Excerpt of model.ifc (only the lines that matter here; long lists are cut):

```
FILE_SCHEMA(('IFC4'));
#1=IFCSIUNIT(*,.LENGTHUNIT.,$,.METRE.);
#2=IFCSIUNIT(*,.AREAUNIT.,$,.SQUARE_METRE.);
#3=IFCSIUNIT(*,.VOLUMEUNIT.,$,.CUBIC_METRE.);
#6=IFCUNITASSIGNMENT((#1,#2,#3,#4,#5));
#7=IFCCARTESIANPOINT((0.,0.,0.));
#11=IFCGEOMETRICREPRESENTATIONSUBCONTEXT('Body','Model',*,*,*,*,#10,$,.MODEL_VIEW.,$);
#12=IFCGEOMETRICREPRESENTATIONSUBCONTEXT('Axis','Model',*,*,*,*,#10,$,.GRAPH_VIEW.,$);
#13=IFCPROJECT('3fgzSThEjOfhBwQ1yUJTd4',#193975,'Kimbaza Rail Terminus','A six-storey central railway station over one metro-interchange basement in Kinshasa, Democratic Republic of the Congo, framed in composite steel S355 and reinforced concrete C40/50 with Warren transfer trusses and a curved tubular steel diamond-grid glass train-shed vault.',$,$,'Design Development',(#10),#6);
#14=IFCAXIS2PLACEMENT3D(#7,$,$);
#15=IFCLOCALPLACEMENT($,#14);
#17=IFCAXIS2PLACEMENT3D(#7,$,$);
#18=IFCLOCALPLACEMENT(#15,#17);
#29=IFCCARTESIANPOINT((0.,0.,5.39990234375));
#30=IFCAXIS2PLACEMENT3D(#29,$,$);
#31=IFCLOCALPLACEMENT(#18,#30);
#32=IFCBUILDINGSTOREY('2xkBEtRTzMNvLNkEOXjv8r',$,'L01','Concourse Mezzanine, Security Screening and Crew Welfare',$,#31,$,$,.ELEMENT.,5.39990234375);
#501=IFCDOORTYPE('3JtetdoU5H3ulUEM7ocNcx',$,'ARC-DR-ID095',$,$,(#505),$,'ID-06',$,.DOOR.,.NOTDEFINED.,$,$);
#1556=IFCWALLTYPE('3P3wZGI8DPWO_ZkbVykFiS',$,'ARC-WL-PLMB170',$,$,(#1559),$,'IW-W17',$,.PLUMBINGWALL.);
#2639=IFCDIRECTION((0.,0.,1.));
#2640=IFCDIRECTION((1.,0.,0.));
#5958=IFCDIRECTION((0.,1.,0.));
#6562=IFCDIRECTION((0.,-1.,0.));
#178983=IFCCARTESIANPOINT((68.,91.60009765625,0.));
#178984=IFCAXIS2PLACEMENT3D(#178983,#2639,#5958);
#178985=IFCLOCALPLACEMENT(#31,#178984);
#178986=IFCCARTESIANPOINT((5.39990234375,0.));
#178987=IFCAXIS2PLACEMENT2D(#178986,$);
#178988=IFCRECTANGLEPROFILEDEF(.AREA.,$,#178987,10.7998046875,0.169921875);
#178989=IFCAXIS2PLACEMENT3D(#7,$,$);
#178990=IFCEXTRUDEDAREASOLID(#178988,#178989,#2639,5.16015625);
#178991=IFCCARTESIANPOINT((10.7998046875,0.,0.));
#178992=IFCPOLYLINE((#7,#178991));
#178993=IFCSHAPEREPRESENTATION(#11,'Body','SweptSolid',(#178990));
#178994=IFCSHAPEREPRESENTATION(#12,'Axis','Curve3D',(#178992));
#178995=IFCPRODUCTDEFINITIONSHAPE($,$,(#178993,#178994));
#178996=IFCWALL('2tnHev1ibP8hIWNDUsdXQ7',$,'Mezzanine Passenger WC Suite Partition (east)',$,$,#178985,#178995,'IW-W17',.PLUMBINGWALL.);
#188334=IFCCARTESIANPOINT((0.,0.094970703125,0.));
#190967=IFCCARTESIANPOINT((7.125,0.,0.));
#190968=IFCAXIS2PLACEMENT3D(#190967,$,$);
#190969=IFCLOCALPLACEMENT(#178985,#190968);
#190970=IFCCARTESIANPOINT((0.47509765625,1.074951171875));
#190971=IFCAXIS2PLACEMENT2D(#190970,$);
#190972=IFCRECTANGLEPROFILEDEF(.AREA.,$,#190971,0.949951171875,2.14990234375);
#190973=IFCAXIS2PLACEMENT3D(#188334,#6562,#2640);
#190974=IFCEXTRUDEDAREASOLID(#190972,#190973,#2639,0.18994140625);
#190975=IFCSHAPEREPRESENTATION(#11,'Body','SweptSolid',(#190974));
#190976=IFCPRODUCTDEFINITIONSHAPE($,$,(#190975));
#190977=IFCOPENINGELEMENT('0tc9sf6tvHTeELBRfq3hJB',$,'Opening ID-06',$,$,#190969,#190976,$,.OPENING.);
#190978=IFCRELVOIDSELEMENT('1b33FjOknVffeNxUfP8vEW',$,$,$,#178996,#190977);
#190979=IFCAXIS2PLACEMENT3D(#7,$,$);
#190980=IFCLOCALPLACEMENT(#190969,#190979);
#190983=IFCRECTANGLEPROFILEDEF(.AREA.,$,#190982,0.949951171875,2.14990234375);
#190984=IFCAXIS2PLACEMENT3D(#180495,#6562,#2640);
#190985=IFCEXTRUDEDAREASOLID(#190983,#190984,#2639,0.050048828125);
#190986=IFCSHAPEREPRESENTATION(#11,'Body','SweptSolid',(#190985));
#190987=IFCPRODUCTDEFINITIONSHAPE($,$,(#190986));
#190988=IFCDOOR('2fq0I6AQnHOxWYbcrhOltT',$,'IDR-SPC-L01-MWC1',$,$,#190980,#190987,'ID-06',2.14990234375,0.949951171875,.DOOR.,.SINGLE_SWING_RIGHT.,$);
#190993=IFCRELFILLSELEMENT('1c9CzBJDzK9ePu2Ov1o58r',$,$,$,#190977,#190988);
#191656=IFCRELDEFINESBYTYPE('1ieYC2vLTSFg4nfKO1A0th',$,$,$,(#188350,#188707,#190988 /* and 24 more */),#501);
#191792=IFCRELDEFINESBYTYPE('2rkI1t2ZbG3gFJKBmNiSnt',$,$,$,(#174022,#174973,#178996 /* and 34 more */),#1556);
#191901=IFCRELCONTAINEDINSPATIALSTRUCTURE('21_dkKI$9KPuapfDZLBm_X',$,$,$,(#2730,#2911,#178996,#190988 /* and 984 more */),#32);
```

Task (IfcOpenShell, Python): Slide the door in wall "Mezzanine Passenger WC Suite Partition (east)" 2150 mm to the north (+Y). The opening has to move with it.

```python
import ifcopenshell
import ifcopenshell.api.geometry
import ifcopenshell.util.placement

model = ifcopenshell.open("model.ifc")

door = model.by_guid("2fq0I6AQnHOxWYbcrhOltT")
opening = door.FillsVoids[0].RelatingOpeningElement
wall = opening.VoidsElements[0].RelatingBuildingElement

wall_matrix = ifcopenshell.util.placement.get_local_placement(wall.ObjectPlacement)
shift = wall_matrix[:3, 0] * 2.15
before = ifcopenshell.util.placement.get_local_placement(door.ObjectPlacement)[:3, 3].copy()

# The door is placed relative to its opening, so it follows when the opening moves.
matrix = ifcopenshell.util.placement.get_local_placement(opening.ObjectPlacement)
matrix[:3, 3] += shift
ifcopenshell.api.geometry.edit_object_placement(
    model, product=opening, matrix=matrix, is_si=False, should_transform_children=True
)

after = ifcopenshell.util.placement.get_local_placement(door.ObjectPlacement)[:3, 3]
print("door moved by", (after - before).round(3) + 0.0)

model.write("model_updated.ifc")
```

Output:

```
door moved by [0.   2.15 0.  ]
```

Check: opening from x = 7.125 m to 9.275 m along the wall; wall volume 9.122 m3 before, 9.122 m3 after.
